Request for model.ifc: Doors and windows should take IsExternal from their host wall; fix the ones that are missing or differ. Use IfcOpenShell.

First a look at what the model holds.

```python
import ifcopenshell
import ifcopenshell.util.element

model = ifcopenshell.open("model.ifc")
print(model.schema)
seen = {}
for e in model.by_type("IfcDoor") + model.by_type("IfcWindow"):
    if not e.FillsVoids:
        continue
    host = e.FillsVoids[0].RelatingOpeningElement.VoidsElements[0].RelatingBuildingElement
    own = ifcopenshell.util.element.get_pset(e, f"Pset_{e.is_a()[3:].removesuffix('StandardCase')}Common", "IsExternal")
    wall = ifcopenshell.util.element.get_pset(host, "Pset_WallCommon", "IsExternal")
    seen[e.is_a(), own, wall] = seen.get((e.is_a(), own, wall), 0) + 1
for (cls, own, wall), count in sorted(seen.items(), key=str):
    print(count, cls, "IsExternal:", own, "| host wall:", wall)
```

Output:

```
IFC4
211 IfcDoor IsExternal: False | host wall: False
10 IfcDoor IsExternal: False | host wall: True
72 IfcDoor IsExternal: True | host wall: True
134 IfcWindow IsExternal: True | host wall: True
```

```python
import ifcopenshell
import ifcopenshell.api.pset
import ifcopenshell.util.element

model = ifcopenshell.open("model.ifc")

count = 0
for ifc_class, pset_name in (("IfcDoor", "Pset_DoorCommon"), ("IfcWindow", "Pset_WindowCommon")):
    for e in model.by_type(ifc_class):
        if not e.FillsVoids:
            continue
        host = e.FillsVoids[0].RelatingOpeningElement.VoidsElements[0].RelatingBuildingElement
        external = ifcopenshell.util.element.get_pset(host, "Pset_WallCommon", "IsExternal")
        if external is None or ifcopenshell.util.element.get_pset(e, pset_name, "IsExternal") == external:
            continue
        pset = ifcopenshell.api.pset.add_pset(model, product=e, name=pset_name)
        ifcopenshell.api.pset.edit_pset(model, pset=pset, properties={"IsExternal": external})
        count += 1

print(count, "updated")

model.write("model_updated.ifc")
```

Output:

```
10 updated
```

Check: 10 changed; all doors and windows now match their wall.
